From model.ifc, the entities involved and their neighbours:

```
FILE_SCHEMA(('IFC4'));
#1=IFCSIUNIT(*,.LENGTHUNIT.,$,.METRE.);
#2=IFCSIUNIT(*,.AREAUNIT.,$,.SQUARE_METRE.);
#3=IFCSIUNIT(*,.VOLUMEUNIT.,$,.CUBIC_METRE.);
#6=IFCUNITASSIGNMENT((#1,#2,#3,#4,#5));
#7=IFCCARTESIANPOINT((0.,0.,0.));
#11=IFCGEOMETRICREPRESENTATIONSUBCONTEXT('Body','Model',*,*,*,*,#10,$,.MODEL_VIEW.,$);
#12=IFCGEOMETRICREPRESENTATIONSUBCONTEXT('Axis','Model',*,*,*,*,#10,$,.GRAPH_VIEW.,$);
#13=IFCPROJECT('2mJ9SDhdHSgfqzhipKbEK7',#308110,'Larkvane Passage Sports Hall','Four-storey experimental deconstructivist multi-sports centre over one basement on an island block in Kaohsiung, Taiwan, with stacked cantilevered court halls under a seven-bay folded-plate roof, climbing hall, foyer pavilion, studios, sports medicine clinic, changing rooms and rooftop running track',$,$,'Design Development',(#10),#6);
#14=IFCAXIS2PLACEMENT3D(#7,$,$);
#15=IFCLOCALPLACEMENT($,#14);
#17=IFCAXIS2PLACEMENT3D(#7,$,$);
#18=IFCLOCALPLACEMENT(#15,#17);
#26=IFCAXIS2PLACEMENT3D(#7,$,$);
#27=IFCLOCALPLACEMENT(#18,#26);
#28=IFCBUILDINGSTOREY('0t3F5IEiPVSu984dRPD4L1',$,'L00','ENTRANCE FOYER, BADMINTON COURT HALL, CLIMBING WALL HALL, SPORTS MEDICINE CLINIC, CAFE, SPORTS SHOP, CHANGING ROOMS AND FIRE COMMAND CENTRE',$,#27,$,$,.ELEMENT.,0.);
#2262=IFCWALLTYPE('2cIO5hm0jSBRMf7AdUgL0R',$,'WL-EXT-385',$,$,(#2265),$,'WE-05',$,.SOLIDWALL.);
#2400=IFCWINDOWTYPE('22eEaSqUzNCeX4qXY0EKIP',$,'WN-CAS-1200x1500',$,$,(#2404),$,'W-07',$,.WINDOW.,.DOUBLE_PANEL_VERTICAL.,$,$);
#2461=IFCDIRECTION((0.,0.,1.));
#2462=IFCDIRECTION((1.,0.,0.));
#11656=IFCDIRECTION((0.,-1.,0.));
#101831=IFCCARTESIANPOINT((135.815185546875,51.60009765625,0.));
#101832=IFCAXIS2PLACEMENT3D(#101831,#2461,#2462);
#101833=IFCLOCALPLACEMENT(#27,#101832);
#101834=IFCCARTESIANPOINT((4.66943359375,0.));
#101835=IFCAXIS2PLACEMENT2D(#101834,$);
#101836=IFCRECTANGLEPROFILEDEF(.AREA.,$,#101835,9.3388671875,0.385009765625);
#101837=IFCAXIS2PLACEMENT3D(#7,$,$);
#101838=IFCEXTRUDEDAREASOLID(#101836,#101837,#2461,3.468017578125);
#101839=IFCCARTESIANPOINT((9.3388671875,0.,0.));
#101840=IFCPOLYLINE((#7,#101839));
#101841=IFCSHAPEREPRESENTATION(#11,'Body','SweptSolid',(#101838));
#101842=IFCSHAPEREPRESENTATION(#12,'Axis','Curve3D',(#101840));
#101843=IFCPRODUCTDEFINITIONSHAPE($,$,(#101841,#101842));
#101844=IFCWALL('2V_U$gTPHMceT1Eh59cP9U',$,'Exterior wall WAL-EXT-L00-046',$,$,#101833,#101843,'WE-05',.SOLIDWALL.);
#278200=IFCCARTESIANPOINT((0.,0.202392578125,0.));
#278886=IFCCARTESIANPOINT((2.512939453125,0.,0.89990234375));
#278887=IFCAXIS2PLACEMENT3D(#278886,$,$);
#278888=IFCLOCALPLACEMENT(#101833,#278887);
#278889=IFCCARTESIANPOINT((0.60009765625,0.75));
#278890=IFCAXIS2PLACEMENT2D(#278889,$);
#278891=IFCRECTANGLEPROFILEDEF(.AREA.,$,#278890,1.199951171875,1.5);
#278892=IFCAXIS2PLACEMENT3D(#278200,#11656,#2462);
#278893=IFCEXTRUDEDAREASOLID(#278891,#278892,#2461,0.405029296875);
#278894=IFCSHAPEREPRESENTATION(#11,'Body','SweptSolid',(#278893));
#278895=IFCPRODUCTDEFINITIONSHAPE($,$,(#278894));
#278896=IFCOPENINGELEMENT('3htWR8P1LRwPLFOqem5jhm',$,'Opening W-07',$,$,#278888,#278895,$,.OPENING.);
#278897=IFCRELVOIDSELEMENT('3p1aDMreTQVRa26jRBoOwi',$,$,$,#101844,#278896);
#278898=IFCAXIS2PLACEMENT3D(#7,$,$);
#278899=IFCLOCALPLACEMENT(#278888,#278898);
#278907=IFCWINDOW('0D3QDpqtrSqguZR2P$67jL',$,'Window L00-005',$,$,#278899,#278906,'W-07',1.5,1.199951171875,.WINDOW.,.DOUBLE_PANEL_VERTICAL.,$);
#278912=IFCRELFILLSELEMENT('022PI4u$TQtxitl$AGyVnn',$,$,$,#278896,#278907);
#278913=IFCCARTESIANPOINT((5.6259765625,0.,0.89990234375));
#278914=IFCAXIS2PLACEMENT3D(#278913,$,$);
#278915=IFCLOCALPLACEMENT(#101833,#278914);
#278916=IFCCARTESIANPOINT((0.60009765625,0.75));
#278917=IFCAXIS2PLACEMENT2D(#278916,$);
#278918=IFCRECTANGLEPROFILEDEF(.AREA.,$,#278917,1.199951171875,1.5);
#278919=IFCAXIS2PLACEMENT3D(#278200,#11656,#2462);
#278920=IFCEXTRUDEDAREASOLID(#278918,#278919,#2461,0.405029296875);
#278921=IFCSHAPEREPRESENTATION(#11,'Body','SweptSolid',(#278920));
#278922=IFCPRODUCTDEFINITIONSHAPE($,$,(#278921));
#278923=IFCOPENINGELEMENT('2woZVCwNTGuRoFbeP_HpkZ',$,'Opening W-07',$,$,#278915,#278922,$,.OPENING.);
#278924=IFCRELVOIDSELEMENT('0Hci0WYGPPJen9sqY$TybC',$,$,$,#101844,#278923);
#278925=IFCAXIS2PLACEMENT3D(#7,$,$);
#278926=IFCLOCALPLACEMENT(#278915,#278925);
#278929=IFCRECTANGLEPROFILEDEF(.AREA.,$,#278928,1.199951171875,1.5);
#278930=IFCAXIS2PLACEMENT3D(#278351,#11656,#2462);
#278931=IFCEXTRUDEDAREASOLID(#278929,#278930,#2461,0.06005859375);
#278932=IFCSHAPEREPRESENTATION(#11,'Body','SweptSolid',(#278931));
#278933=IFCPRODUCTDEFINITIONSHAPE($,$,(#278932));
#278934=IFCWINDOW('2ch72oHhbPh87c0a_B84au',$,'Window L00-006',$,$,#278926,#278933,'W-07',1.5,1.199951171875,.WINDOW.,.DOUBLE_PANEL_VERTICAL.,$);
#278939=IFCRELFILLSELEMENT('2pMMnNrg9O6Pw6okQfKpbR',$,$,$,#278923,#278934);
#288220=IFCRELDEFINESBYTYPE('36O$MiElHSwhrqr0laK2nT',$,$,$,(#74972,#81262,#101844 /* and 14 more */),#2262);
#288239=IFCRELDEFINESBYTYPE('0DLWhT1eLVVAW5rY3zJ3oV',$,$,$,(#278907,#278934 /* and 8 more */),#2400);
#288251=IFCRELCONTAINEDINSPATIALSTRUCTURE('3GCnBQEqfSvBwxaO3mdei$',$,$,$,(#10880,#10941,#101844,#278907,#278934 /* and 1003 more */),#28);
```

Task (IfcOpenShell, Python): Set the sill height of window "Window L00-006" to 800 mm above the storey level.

```python
import numpy as np
import ifcopenshell
import ifcopenshell.api.geometry
import ifcopenshell.geom
import ifcopenshell.util.element
import ifcopenshell.util.placement
import ifcopenshell.util.shape
import ifcopenshell.util.unit

model = ifcopenshell.open("model.ifc")
unit_scale = ifcopenshell.util.unit.calculate_unit_scale(model)

window = model.by_guid("2ch72oHhbPh87c0a_B84au")
opening = window.FillsVoids[0].RelatingOpeningElement
storey = ifcopenshell.util.element.get_container(window, ifc_class="IfcBuildingStorey")
level = ifcopenshell.util.placement.get_local_placement(storey.ObjectPlacement)[2, 3]

# The opening's origin need not be at the sill, so measure its lowest point.
shape = ifcopenshell.geom.create_shape(ifcopenshell.geom.settings(), opening)
bottom = ifcopenshell.util.shape.get_shape_bottom_elevation(shape, shape.geometry) / unit_scale
dz = level + 0.8 / unit_scale - bottom

shift = np.array([0.0, 0.0, dz])
# The window is placed relative to its opening, so it follows when the opening moves.
matrix = ifcopenshell.util.placement.get_local_placement(opening.ObjectPlacement)
matrix[:3, 3] += shift
ifcopenshell.api.geometry.edit_object_placement(
    model, product=opening, matrix=matrix, is_si=False, should_transform_children=True
)

print(f"moved by {dz * unit_scale:+.3f} m")

model.write("model_rev.ifc")
```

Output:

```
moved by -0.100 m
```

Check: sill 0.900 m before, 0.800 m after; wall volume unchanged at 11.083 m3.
